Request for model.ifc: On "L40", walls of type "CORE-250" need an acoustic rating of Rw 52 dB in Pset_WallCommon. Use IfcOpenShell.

First a look at what the model holds.

```python
import ifcopenshell
import ifcopenshell.util.element

model = ifcopenshell.open("model.ifc")
print(model.schema)
storey = next(s for s in model.by_type("IfcBuildingStorey") if s.Name == "L40")
walls = [e for e in ifcopenshell.util.element.get_decomposition(storey) if e.is_a("IfcWall")]
seen = {}
for e in walls:
    element_type = ifcopenshell.util.element.get_type(e)
    key = (element_type.Name if element_type != e and element_type else None, ifcopenshell.util.element.get_pset(e, "Pset_WallCommon", "AcousticRating"))
    seen[key] = seen.get(key, 0) + 1
for (name, value), count in sorted(seen.items(), key=str):
    print(count, "x", name, "|", value)
```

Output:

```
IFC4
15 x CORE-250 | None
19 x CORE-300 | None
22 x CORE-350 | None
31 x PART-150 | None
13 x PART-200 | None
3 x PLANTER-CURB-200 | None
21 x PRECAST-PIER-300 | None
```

```python
import ifcopenshell
import ifcopenshell.api.pset
import ifcopenshell.util.element

model = ifcopenshell.open("model.ifc")

storey = next(s for s in model.by_type("IfcBuildingStorey") if s.Name == "L40")
walls = [e for e in ifcopenshell.util.element.get_decomposition(storey) if e.is_a("IfcWall")]

count = 0
for e in walls:
    element_type = ifcopenshell.util.element.get_type(e)
    if element_type in (None, e) or element_type.Name != "CORE-250":
        continue
    found = ifcopenshell.util.element.get_pset(e, "Pset_WallCommon", should_inherit=False)
    if found:
        pset = model.by_id(found["id"])
        if len(ifcopenshell.util.element.get_elements_by_pset(pset)) > 1:
            pset = ifcopenshell.api.pset.unshare_pset(model, products=[e], pset=pset)[0]
    else:
        pset = ifcopenshell.api.pset.add_pset(model, product=e, name="Pset_WallCommon")
    ifcopenshell.api.pset.edit_pset(model, pset=pset, properties={"AcousticRating": "Rw 52 dB"})
    count += 1

print(count, "walls updated")

model.write("model_updated.ifc")
```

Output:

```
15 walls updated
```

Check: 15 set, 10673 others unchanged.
